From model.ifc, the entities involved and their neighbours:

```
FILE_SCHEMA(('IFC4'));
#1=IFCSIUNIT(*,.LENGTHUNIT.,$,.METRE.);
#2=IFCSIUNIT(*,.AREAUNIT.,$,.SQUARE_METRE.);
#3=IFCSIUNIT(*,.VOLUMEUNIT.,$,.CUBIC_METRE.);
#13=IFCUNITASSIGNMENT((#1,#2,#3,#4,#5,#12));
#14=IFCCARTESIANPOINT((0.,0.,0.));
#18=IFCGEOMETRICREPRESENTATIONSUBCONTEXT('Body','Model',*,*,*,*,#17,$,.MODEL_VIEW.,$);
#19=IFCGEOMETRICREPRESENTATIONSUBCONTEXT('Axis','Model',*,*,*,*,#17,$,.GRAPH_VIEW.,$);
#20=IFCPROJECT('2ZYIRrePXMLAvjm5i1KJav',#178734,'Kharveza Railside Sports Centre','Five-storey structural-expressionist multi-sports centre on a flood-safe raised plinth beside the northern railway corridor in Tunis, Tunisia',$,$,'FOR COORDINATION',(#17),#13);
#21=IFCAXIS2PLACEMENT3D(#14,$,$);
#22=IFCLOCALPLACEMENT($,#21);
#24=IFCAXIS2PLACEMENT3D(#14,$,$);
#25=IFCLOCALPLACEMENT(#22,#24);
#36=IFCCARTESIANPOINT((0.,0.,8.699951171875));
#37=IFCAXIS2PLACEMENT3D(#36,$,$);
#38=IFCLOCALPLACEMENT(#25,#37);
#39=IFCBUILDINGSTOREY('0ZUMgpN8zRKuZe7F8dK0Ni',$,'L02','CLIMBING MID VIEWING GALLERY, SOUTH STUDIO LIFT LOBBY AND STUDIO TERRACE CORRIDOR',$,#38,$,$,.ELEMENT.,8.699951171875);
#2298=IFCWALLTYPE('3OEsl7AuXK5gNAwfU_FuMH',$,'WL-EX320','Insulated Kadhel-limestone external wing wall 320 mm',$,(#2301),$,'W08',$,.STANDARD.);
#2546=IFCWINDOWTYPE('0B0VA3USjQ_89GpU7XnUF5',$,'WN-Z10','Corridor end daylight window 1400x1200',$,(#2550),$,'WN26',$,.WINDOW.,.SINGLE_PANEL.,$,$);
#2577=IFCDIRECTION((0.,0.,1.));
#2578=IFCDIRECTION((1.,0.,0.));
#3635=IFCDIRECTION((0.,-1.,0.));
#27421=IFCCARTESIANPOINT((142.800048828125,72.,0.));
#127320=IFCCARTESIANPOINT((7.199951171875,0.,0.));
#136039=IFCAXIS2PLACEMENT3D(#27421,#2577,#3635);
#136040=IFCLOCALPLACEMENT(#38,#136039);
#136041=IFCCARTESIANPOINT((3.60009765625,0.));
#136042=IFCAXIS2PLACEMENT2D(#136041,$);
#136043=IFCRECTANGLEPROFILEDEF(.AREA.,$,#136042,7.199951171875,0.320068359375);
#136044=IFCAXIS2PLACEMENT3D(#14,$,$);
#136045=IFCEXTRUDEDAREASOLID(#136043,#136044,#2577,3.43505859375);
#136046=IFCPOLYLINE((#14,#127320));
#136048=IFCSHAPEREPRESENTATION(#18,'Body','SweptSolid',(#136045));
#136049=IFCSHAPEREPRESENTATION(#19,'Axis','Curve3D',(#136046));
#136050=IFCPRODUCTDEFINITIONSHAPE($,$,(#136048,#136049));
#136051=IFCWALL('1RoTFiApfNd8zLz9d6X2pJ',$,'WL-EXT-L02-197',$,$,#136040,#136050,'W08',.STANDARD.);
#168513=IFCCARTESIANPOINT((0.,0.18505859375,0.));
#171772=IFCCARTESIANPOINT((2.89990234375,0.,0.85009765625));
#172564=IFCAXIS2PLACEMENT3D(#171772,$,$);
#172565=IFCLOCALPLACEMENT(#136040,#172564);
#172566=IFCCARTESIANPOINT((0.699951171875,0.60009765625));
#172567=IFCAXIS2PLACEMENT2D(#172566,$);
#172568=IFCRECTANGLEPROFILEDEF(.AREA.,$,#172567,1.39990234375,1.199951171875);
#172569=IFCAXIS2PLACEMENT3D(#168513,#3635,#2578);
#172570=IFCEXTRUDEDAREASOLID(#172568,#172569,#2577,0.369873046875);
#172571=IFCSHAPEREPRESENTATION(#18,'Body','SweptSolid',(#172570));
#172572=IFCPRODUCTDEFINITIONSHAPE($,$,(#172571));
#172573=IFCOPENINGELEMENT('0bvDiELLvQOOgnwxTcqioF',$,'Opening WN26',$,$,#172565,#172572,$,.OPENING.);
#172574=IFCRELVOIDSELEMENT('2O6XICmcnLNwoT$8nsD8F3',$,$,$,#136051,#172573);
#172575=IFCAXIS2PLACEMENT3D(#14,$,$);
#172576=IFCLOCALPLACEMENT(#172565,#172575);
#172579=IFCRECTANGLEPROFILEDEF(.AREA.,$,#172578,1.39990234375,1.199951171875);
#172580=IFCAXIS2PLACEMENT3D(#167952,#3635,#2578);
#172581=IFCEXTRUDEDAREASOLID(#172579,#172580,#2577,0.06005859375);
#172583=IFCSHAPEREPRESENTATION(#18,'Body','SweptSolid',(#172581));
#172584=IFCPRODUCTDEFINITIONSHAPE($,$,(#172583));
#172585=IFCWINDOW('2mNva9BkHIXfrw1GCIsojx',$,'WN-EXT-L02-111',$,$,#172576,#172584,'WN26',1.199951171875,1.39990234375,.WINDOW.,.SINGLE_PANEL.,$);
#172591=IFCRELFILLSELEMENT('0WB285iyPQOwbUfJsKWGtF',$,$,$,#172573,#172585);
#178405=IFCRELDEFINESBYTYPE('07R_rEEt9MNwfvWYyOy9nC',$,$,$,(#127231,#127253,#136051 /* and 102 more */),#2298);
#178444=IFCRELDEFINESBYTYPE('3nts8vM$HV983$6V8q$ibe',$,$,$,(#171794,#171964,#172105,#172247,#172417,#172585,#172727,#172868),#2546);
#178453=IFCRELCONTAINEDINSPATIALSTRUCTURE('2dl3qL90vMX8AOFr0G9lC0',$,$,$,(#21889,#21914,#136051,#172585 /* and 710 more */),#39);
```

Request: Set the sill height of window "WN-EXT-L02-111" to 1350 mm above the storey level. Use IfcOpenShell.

```python
import numpy as np
import ifcopenshell
import ifcopenshell.api.geometry
import ifcopenshell.geom
import ifcopenshell.util.element
import ifcopenshell.util.placement
import ifcopenshell.util.shape
import ifcopenshell.util.unit

model = ifcopenshell.open("model.ifc")
unit_scale = ifcopenshell.util.unit.calculate_unit_scale(model)

window = model.by_guid("2mNva9BkHIXfrw1GCIsojx")
opening = window.FillsVoids[0].RelatingOpeningElement
storey = ifcopenshell.util.element.get_container(window, ifc_class="IfcBuildingStorey")
level = ifcopenshell.util.placement.get_local_placement(storey.ObjectPlacement)[2, 3]

# The opening's origin need not be at the sill, so measure its lowest point.
shape = ifcopenshell.geom.create_shape(ifcopenshell.geom.settings(), opening)
bottom = ifcopenshell.util.shape.get_shape_bottom_elevation(shape, shape.geometry) / unit_scale
dz = level + 1.35 - bottom

shift = np.array([0.0, 0.0, dz])
# The window is placed relative to its opening, so it follows when the opening moves.
matrix = ifcopenshell.util.placement.get_local_placement(opening.ObjectPlacement)
matrix[:3, 3] += shift
ifcopenshell.api.geometry.edit_object_placement(
    model, product=opening, matrix=matrix, is_si=False, should_transform_children=True
)

print(f"moved by {dz * unit_scale:+.3f} m")

model.write("model_rev.ifc")
```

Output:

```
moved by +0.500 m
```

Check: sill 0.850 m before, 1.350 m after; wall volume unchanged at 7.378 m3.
